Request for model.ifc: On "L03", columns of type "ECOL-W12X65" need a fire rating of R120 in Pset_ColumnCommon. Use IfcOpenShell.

First a look at what the model holds.

```python
import ifcopenshell
import ifcopenshell.util.element

model = ifcopenshell.open("model.ifc")
print(model.schema)
storey = next(s for s in model.by_type("IfcBuildingStorey") if s.Name == "L03")
columns = [e for e in ifcopenshell.util.element.get_decomposition(storey) if e.is_a("IfcColumn")]
seen = {}
for e in columns:
    element_type = ifcopenshell.util.element.get_type(e)
    key = (element_type.Name if element_type != e and element_type else None, ifcopenshell.util.element.get_pset(e, "Pset_ColumnCommon", "FireRating"))
    seen[key] = seen.get(key, 0) + 1
for (name, value), count in sorted(seen.items(), key=str):
    print(count, "x", name, "|", value)
```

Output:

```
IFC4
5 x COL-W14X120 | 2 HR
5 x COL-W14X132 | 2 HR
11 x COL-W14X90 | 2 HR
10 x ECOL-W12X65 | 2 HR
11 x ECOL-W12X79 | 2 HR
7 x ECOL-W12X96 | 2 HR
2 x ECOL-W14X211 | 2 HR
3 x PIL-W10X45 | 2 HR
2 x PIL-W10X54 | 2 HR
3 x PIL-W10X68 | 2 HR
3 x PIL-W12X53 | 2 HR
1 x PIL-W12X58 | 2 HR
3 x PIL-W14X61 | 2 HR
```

```python
import ifcopenshell
import ifcopenshell.api.pset
import ifcopenshell.util.element

model = ifcopenshell.open("model.ifc")

storey = next(s for s in model.by_type("IfcBuildingStorey") if s.Name == "L03")
columns = [e for e in ifcopenshell.util.element.get_decomposition(storey) if e.is_a("IfcColumn")]

count = 0
for e in columns:
    element_type = ifcopenshell.util.element.get_type(e)
    if element_type in (None, e) or element_type.Name != "ECOL-W12X65":
        continue
    # add_pset returns the element's existing set when there is one.
    pset = ifcopenshell.api.pset.add_pset(model, product=e, name="Pset_ColumnCommon")
    ifcopenshell.api.pset.edit_pset(model, pset=pset, properties={"FireRating": "R120"})
    count += 1

print(count, "columns updated")

model.write("model_v2.ifc")
```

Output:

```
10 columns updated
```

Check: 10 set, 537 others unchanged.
